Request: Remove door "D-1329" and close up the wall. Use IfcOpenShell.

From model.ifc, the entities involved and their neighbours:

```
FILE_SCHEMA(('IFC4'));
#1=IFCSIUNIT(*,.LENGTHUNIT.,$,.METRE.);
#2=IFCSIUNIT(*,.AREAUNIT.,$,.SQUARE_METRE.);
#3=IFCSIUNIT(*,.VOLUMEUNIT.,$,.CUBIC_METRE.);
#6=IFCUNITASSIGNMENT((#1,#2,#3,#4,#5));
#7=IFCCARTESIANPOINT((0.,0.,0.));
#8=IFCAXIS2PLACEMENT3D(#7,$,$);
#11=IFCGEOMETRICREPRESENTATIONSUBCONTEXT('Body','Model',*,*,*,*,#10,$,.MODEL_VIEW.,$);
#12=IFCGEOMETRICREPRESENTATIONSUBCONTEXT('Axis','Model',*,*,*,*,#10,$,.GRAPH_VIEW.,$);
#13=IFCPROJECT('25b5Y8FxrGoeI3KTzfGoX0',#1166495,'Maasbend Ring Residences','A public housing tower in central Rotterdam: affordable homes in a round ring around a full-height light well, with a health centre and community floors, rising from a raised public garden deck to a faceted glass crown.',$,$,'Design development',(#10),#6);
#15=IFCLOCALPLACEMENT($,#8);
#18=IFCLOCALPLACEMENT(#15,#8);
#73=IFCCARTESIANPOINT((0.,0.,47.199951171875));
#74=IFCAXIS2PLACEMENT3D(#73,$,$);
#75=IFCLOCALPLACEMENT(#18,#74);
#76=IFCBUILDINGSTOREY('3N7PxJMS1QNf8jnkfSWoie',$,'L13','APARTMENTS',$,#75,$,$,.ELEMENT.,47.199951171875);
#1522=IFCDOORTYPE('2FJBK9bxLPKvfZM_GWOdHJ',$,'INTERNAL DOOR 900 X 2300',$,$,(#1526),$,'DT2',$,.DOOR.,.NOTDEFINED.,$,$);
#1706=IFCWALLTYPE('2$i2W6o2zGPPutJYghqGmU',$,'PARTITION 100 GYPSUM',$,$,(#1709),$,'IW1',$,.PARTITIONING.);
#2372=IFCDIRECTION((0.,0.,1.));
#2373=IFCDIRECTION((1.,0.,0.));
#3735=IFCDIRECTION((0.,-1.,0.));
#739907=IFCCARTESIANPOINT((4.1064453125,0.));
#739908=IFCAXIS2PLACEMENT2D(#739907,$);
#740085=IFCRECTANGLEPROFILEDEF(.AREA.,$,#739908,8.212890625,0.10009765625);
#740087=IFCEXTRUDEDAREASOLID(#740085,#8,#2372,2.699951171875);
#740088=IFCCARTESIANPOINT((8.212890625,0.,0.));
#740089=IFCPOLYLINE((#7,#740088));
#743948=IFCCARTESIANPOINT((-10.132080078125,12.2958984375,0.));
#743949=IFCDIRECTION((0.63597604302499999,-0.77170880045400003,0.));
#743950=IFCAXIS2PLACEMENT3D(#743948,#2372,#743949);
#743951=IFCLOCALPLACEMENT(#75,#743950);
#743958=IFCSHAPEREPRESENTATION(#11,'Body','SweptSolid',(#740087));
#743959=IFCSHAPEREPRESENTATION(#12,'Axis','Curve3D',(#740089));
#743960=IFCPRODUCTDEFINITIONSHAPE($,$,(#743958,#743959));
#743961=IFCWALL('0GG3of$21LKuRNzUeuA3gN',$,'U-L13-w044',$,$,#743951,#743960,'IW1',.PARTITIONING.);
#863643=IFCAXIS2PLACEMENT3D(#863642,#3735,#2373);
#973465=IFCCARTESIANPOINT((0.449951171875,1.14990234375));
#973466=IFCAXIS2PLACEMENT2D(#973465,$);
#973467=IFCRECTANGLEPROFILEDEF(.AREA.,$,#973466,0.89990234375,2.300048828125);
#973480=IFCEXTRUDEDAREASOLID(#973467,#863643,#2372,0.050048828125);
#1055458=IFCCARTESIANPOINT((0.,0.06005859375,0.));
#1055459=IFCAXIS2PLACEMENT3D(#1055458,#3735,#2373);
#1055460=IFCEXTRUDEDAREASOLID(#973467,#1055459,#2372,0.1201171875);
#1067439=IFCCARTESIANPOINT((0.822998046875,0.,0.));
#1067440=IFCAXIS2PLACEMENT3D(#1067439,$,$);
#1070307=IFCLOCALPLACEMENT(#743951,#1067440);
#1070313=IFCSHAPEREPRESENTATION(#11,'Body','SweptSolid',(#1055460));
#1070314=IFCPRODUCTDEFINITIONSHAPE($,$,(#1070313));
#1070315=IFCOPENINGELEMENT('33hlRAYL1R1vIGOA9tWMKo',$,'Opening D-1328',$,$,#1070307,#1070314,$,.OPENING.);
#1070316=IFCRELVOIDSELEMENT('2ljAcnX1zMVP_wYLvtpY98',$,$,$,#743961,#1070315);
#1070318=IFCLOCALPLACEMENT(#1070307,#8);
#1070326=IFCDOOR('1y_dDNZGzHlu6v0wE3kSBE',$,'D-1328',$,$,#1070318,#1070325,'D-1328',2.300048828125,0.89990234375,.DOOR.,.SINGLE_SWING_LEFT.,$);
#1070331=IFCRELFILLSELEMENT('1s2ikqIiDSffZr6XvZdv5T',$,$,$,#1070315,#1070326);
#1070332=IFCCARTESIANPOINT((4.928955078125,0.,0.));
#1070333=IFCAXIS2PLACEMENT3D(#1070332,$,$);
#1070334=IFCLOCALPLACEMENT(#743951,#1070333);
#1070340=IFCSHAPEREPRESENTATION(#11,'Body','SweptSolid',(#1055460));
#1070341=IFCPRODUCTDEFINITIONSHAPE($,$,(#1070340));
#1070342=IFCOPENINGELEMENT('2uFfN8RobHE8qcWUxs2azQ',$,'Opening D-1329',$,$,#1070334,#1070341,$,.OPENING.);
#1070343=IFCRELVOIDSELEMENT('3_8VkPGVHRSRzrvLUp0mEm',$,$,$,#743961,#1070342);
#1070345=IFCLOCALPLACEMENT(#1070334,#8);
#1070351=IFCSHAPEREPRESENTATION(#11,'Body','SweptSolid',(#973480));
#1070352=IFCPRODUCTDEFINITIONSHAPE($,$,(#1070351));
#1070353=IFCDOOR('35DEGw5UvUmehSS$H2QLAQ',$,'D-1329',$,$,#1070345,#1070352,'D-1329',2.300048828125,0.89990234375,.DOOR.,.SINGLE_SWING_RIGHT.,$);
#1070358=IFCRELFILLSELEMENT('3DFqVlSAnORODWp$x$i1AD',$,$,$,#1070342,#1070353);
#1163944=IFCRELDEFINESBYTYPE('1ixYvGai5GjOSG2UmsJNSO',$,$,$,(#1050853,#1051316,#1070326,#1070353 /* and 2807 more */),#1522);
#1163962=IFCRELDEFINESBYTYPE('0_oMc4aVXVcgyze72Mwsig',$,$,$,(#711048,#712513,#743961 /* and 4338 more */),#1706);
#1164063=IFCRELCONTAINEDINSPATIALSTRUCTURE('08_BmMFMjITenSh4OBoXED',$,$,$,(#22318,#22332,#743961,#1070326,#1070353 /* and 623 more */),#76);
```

```python
import ifcopenshell
import ifcopenshell.api.feature
import ifcopenshell.api.root
import ifcopenshell.geom
import ifcopenshell.util.shape

model = ifcopenshell.open("model.ifc")
settings = ifcopenshell.geom.settings()


def volume(element):
    """Net volume in cubic metres, openings subtracted."""
    shape = ifcopenshell.geom.create_shape(settings, element)
    return ifcopenshell.util.shape.get_volume(shape.geometry)


door = model.by_id(1070353)
opening = door.FillsVoids[0].RelatingOpeningElement
wall = opening.VoidsElements[0].RelatingBuildingElement
before = volume(wall)

ifcopenshell.api.root.remove_product(model, product=door)
ifcopenshell.api.feature.remove_feature(model, feature=opening)

after = volume(wall)

print(f"wall volume {before:.3f} -> {after:.3f} m3")

model.write("model-out.ifc")
```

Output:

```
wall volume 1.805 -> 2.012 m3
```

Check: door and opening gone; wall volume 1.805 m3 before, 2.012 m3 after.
